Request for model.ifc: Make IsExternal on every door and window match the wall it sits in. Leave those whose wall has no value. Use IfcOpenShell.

First a look at what the model holds.

```python
import ifcopenshell
import ifcopenshell.util.element

model = ifcopenshell.open("model.ifc")
print(model.schema)
seen = {}
for e in model.by_type("IfcDoor") + model.by_type("IfcWindow"):
    if not e.FillsVoids:
        continue
    host = e.FillsVoids[0].RelatingOpeningElement.VoidsElements[0].RelatingBuildingElement
    own = ifcopenshell.util.element.get_pset(e, f"Pset_{e.is_a()[3:].removesuffix('StandardCase')}Common", "IsExternal")
    wall = ifcopenshell.util.element.get_pset(host, "Pset_WallCommon", "IsExternal")
    seen[e.is_a(), own, wall] = seen.get((e.is_a(), own, wall), 0) + 1
for (cls, own, wall), count in sorted(seen.items(), key=str):
    print(count, cls, "IsExternal:", own, "| host wall:", wall)
```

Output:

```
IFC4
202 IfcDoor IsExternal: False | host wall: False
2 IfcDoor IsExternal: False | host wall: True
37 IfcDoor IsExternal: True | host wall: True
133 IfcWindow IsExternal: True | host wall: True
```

```python
import ifcopenshell
import ifcopenshell.api.pset
import ifcopenshell.util.element

model = ifcopenshell.open("model.ifc")

count = 0
for ifc_class, pset_name in (("IfcDoor", "Pset_DoorCommon"), ("IfcWindow", "Pset_WindowCommon")):
    for e in model.by_type(ifc_class):
        if not e.FillsVoids:
            continue
        host = e.FillsVoids[0].RelatingOpeningElement.VoidsElements[0].RelatingBuildingElement
        external = ifcopenshell.util.element.get_pset(host, "Pset_WallCommon", "IsExternal")
        if external is None or ifcopenshell.util.element.get_pset(e, pset_name, "IsExternal") == external:
            continue
        pset = ifcopenshell.api.pset.add_pset(model, product=e, name=pset_name)
        ifcopenshell.api.pset.edit_pset(model, pset=pset, properties={"IsExternal": external})
        count += 1

print(count, "updated")

model.write("model_updated.ifc")
```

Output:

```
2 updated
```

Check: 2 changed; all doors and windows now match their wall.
